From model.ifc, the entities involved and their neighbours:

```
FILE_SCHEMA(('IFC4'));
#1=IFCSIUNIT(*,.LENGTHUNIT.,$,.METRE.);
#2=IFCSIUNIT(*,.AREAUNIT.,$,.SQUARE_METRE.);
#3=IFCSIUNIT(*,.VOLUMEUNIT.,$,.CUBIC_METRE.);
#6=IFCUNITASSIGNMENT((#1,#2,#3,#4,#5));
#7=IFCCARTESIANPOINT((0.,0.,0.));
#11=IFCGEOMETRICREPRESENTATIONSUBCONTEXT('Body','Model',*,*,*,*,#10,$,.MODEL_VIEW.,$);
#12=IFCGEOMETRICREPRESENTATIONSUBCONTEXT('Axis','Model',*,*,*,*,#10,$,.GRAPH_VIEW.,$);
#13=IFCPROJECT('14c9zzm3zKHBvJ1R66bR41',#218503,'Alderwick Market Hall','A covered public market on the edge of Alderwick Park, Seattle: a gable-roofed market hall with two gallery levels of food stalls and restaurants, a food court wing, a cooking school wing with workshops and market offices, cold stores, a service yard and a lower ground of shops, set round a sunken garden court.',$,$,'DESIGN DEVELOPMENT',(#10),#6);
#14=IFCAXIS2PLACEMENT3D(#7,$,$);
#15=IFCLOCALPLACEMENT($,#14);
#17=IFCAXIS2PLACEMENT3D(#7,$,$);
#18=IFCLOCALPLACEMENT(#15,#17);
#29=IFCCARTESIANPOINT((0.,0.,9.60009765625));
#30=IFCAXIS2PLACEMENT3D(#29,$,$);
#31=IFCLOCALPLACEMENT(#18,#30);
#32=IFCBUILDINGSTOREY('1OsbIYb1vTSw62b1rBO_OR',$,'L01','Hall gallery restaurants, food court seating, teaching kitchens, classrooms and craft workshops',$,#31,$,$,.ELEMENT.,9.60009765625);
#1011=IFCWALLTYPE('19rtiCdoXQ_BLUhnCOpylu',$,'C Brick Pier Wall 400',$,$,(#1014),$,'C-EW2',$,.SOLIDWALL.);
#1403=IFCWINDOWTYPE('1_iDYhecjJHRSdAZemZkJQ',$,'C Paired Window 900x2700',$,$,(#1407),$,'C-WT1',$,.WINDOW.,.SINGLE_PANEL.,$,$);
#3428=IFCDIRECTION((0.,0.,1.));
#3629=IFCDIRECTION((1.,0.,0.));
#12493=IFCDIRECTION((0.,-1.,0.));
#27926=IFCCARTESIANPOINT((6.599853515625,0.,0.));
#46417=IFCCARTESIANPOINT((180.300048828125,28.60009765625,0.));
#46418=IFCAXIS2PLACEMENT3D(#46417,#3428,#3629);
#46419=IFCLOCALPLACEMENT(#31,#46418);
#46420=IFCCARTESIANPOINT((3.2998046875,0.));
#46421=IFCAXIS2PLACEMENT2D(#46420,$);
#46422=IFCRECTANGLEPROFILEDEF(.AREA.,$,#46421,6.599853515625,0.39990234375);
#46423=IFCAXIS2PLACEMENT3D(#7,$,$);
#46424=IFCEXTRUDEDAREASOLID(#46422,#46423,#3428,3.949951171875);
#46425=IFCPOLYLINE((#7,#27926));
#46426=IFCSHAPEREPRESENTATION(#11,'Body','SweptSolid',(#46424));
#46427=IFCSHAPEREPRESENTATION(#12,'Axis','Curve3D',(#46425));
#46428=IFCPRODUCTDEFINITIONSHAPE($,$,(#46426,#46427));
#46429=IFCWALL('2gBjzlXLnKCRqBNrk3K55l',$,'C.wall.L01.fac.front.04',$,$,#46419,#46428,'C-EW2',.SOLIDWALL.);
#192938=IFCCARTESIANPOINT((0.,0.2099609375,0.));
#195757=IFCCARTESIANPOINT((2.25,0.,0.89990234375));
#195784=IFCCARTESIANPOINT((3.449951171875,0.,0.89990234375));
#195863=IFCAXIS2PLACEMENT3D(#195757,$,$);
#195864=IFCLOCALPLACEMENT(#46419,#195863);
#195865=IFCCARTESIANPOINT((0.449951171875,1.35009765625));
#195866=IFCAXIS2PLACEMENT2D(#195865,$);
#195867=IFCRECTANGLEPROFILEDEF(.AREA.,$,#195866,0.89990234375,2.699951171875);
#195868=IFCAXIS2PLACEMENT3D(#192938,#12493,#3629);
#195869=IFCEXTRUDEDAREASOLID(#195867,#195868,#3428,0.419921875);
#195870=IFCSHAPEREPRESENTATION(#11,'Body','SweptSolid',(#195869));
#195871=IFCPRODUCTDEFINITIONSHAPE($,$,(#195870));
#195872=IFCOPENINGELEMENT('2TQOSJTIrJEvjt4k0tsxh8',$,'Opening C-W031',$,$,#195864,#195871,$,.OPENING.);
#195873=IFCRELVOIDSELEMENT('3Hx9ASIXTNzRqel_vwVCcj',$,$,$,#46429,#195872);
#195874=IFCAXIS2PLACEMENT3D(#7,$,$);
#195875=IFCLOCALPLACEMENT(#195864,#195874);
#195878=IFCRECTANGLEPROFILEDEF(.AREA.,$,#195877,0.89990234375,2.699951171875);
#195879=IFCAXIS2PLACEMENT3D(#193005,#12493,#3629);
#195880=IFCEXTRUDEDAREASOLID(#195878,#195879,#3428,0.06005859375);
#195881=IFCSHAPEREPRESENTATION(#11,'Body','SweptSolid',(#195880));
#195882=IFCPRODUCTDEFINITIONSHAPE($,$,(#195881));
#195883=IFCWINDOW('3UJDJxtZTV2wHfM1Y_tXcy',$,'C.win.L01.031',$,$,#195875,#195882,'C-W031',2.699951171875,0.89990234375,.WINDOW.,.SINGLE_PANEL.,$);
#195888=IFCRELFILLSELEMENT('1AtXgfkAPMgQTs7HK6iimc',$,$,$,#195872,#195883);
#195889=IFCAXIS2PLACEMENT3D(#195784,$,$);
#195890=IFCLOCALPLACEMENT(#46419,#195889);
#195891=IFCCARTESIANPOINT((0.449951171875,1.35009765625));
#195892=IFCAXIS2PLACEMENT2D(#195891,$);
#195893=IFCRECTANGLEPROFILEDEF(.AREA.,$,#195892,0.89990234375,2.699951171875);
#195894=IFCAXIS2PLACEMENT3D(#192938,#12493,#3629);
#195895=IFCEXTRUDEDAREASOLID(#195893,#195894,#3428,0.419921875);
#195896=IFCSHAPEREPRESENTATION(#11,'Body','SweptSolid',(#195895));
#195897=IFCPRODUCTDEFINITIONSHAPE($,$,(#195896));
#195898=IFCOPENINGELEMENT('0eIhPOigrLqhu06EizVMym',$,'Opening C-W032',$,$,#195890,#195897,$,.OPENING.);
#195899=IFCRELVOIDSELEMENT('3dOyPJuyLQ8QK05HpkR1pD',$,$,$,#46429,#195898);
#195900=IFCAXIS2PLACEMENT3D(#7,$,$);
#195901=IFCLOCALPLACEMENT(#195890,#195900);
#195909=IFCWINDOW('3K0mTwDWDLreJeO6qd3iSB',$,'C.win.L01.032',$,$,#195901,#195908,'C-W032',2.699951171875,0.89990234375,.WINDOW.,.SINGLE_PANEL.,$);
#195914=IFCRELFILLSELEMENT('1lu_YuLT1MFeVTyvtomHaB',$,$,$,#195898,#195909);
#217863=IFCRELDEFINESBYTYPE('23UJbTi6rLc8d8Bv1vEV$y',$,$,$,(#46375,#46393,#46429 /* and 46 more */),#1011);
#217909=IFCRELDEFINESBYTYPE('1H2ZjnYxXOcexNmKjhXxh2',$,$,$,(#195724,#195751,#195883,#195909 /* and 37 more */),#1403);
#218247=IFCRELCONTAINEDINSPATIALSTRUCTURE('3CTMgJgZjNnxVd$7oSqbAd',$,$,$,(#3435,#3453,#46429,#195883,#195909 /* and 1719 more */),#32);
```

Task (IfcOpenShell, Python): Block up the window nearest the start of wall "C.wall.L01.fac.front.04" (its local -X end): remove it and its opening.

```python
import ifcopenshell
import ifcopenshell.api.feature
import ifcopenshell.api.root
import ifcopenshell.geom
import ifcopenshell.util.shape

model = ifcopenshell.open("model.ifc")
settings = ifcopenshell.geom.settings()


def volume(element):
    """Net volume in cubic metres, openings subtracted."""
    shape = ifcopenshell.geom.create_shape(settings, element)
    return ifcopenshell.util.shape.get_volume(shape.geometry)


window = model.by_id(195883)
opening = window.FillsVoids[0].RelatingOpeningElement
wall = opening.VoidsElements[0].RelatingBuildingElement
before = volume(wall)

ifcopenshell.api.root.remove_product(model, product=window)
ifcopenshell.api.feature.remove_feature(model, feature=opening)

after = volume(wall)

print(f"wall volume {before:.3f} -> {after:.3f} m3")

model.write("model_updated.ifc")
```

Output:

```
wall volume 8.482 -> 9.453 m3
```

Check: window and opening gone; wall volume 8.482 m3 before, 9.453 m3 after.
